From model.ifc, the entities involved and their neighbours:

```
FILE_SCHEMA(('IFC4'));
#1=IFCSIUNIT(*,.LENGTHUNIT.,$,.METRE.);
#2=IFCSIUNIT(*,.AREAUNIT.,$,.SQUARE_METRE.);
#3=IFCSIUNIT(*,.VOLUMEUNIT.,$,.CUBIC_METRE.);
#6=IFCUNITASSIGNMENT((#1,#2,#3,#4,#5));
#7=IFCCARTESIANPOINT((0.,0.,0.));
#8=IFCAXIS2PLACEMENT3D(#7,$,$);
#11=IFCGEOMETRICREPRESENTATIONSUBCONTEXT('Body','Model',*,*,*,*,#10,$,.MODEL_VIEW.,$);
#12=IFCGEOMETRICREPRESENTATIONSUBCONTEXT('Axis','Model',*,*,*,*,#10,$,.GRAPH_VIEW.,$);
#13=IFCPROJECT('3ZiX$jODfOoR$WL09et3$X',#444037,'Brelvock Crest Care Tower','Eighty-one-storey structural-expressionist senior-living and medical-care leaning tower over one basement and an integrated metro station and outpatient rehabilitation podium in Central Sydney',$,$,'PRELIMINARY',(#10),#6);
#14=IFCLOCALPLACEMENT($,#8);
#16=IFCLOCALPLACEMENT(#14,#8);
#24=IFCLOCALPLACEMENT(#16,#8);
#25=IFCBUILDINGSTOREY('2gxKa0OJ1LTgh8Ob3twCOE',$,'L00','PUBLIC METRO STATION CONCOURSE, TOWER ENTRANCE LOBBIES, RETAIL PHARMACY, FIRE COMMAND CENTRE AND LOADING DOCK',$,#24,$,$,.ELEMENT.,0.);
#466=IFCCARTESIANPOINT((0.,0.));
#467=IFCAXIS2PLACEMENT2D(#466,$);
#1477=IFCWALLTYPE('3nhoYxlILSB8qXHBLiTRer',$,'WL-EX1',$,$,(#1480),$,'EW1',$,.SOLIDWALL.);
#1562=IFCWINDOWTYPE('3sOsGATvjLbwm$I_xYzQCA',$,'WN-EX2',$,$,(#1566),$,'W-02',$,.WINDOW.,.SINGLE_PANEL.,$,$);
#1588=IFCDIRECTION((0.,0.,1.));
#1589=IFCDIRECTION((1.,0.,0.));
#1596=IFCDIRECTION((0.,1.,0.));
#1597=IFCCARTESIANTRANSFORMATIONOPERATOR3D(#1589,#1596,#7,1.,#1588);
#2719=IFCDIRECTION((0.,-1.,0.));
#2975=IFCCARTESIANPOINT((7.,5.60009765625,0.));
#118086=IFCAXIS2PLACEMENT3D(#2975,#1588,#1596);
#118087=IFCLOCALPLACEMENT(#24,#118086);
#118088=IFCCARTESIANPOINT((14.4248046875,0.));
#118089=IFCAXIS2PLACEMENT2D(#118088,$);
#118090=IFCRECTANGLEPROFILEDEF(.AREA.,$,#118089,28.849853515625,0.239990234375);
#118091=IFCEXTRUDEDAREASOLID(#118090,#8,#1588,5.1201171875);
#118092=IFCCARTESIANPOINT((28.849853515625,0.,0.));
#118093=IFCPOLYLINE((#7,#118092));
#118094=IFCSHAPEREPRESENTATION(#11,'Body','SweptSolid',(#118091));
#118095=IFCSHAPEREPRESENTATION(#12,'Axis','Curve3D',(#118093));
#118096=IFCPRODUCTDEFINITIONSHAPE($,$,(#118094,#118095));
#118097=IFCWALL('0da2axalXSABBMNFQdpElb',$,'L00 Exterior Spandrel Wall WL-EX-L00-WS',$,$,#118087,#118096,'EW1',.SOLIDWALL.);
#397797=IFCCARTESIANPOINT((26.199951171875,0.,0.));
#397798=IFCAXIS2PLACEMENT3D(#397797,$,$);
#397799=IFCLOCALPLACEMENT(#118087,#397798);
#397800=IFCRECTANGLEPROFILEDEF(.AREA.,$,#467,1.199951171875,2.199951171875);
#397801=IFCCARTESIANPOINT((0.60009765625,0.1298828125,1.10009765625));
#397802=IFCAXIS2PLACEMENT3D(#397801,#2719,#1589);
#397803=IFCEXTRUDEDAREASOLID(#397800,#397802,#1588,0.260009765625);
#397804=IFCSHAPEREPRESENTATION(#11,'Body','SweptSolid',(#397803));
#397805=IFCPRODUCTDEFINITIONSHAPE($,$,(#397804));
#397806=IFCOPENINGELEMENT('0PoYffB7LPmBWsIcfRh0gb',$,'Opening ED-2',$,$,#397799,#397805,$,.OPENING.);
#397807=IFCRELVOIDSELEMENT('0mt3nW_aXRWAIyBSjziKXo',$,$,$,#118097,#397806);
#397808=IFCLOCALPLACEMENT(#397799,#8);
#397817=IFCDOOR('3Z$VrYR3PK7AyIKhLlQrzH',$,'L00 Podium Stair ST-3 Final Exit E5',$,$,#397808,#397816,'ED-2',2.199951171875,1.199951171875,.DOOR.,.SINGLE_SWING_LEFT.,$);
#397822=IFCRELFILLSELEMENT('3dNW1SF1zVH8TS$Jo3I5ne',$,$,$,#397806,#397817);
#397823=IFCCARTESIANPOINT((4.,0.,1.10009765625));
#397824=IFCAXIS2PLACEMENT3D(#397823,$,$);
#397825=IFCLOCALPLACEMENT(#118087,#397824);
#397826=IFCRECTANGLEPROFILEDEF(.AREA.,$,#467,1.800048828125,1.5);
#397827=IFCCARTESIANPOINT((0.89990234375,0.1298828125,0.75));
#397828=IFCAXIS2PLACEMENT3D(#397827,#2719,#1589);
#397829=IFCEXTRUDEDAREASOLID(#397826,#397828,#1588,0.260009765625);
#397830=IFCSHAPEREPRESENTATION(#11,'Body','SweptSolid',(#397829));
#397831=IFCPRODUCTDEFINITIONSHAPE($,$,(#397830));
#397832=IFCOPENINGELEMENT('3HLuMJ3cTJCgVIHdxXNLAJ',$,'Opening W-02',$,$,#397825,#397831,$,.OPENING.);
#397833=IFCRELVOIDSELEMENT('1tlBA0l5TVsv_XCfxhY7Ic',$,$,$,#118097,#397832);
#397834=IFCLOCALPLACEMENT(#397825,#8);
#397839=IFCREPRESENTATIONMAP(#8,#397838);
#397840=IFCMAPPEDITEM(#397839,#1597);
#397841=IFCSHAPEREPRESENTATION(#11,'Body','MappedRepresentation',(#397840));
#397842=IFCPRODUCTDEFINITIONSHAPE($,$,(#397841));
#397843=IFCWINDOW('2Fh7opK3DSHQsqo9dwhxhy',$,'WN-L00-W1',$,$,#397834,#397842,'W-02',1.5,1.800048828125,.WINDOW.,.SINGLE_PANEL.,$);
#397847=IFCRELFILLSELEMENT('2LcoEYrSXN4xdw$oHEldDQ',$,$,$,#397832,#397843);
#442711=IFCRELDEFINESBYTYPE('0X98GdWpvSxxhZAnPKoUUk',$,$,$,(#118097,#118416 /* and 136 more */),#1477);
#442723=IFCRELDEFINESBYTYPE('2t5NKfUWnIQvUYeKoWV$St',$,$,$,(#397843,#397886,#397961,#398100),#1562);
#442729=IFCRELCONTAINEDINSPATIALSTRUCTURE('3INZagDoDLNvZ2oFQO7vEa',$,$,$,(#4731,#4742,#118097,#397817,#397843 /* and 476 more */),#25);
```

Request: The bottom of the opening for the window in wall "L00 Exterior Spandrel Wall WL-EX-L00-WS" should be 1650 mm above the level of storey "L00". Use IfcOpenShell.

```python
import numpy as np
import ifcopenshell
import ifcopenshell.api.geometry
import ifcopenshell.geom
import ifcopenshell.util.element
import ifcopenshell.util.placement
import ifcopenshell.util.shape
import ifcopenshell.util.unit

model = ifcopenshell.open("model.ifc")
unit_scale = ifcopenshell.util.unit.calculate_unit_scale(model)

window = model.by_guid("2Fh7opK3DSHQsqo9dwhxhy")
opening = window.FillsVoids[0].RelatingOpeningElement
storey = ifcopenshell.util.element.get_container(window, ifc_class="IfcBuildingStorey")
level = ifcopenshell.util.placement.get_local_placement(storey.ObjectPlacement)[2, 3]

# The opening's origin need not be at the sill, so measure its lowest point.
shape = ifcopenshell.geom.create_shape(ifcopenshell.geom.settings(), opening)
bottom = ifcopenshell.util.shape.get_shape_bottom_elevation(shape, shape.geometry) / unit_scale
dz = level + 1.65 / unit_scale - bottom

shift = np.array([0.0, 0.0, dz])
# The window is placed relative to its opening, so it follows when the opening moves.
matrix = ifcopenshell.util.placement.get_local_placement(opening.ObjectPlacement)
matrix[:3, 3] += shift
ifcopenshell.api.geometry.edit_object_placement(
    model, product=opening, matrix=matrix, is_si=False, should_transform_children=True
)

print(f"moved by {dz * unit_scale:+.3f} m")

model.write("model_updated.ifc")
```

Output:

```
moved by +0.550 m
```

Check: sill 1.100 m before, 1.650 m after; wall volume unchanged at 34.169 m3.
